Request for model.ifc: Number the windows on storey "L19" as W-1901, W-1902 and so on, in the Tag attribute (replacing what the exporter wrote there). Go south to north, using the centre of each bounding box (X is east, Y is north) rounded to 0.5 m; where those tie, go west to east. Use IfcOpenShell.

First a look at what the model holds.

```python
import ifcopenshell
import ifcopenshell.util.element
import ifcopenshell.util.placement

model = ifcopenshell.open("model.ifc")
print(model.schema)
storey = next(s for s in model.by_type("IfcBuildingStorey") if s.Name == "L19")
windows = [e for e in ifcopenshell.util.element.get_decomposition(storey) if e.is_a("IfcWindow")]
for e in sorted(windows, key=lambda e: e.id()):
    origin = ifcopenshell.util.placement.get_local_placement(e.ObjectPlacement)[:3, 3]
    print(e.id(), e.Tag, e.Name, origin.round(2) + 0.0, sep=" | ")
```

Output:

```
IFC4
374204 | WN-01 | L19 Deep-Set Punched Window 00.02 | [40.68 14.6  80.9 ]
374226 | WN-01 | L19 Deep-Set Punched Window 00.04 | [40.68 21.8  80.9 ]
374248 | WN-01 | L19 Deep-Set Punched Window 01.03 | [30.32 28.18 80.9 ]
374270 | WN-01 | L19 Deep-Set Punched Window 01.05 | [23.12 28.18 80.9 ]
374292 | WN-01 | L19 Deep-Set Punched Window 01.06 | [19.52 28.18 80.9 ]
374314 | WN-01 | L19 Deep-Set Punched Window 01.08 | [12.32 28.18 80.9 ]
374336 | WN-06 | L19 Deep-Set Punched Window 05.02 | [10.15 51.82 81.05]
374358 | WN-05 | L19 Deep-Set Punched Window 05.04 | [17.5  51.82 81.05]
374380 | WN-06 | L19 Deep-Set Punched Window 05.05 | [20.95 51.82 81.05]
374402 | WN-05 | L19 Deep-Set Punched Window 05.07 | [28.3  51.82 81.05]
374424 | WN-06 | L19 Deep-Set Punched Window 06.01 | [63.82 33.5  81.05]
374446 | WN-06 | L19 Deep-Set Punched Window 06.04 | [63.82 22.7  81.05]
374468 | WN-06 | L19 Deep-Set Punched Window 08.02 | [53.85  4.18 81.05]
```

```python
import ifcopenshell
import ifcopenshell.geom
import ifcopenshell.util.element
import ifcopenshell.util.shape

model = ifcopenshell.open("model.ifc")
settings = ifcopenshell.geom.settings()
settings.set("use-world-coords", True)


def centre(element):
    shape = ifcopenshell.geom.create_shape(settings, element)
    return ifcopenshell.util.shape.get_bbox_centroid(shape.geometry)


storey = next(s for s in model.by_type("IfcBuildingStorey") if s.Name == "L19")
windows = [e for e in ifcopenshell.util.element.get_decomposition(storey) if e.is_a("IfcWindow")]

# Insertion points can sit at a corner or the storey origin, so sort by the geometry (in metres).
centres = {e: centre(e) for e in windows}
windows.sort(key=lambda e: (round(centres[e][1] / 0.5), centres[e][0]))

for i, e in enumerate(windows, start=1):
    number = f"W-19{i:02d}"
    e.Tag = number
    print(e.id(), number)

model.write("model-out.ifc")
```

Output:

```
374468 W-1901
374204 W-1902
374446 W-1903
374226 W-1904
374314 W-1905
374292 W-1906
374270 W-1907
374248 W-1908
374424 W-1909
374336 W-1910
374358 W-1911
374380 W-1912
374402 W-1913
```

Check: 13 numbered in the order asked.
